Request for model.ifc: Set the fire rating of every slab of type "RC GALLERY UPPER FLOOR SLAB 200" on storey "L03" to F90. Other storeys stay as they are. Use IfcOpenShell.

First a look at what the model holds.

```python
import ifcopenshell
import ifcopenshell.util.element

model = ifcopenshell.open("model.ifc")
print(model.schema)
storey = next(s for s in model.by_type("IfcBuildingStorey") if s.Name == "L03")
slabs = [e for e in ifcopenshell.util.element.get_decomposition(storey) if e.is_a("IfcSlab")]
seen = {}
for e in slabs:
    element_type = ifcopenshell.util.element.get_type(e)
    key = (element_type.Name if element_type != e and element_type else None, ifcopenshell.util.element.get_pset(e, "Pset_SlabCommon", "FireRating"))
    seen[key] = seen.get(key, 0) + 1
for (name, value), count in sorted(seen.items(), key=str):
    print(count, "x", name, "|", value)
```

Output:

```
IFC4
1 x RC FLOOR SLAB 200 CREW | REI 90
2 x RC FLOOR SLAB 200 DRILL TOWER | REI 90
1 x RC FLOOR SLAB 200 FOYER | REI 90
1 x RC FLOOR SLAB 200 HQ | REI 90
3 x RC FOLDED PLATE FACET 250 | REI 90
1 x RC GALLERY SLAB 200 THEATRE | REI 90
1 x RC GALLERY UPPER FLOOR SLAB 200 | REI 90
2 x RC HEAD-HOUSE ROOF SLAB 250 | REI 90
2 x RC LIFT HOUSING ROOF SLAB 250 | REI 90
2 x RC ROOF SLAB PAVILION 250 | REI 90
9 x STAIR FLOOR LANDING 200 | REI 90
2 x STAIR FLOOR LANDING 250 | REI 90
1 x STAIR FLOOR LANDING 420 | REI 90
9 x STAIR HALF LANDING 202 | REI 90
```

```python
import ifcopenshell
import ifcopenshell.api.pset
import ifcopenshell.util.element

model = ifcopenshell.open("model.ifc")

storey = next(s for s in model.by_type("IfcBuildingStorey") if s.Name == "L03")
slabs = [e for e in ifcopenshell.util.element.get_decomposition(storey) if e.is_a("IfcSlab")]

count = 0
for e in slabs:
    element_type = ifcopenshell.util.element.get_type(e)
    if element_type in (None, e) or element_type.Name != "RC GALLERY UPPER FLOOR SLAB 200":
        continue
    # add_pset returns the element's existing set when there is one.
    pset = ifcopenshell.api.pset.add_pset(model, product=e, name="Pset_SlabCommon")
    ifcopenshell.api.pset.edit_pset(model, pset=pset, properties={"FireRating": "F90"})
    count += 1

print(count, "slabs updated")

model.write("model_v2.ifc")
```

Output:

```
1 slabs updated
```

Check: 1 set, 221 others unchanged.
